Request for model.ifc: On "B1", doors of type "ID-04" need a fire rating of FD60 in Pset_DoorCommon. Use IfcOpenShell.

First a look at what the model holds.

```python
import ifcopenshell
import ifcopenshell.util.element

model = ifcopenshell.open("model.ifc")
print(model.schema)
storey = next(s for s in model.by_type("IfcBuildingStorey") if s.Name == "B1")
doors = [e for e in ifcopenshell.util.element.get_decomposition(storey) if e.is_a("IfcDoor")]
seen = {}
for e in doors:
    element_type = ifcopenshell.util.element.get_type(e)
    key = (element_type.Name if element_type != e and element_type else None, ifcopenshell.util.element.get_pset(e, "Pset_DoorCommon", "FireRating"))
    seen[key] = seen.get(key, 0) + 1
for (name, value), count in sorted(seen.items(), key=str):
    print(count, "x", name, "|", value)
```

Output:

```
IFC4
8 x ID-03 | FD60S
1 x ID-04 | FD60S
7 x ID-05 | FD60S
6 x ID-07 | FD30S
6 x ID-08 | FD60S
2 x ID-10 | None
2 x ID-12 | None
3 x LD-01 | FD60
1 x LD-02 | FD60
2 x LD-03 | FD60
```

```python
import ifcopenshell
import ifcopenshell.api.pset
import ifcopenshell.util.element

model = ifcopenshell.open("model.ifc")

storey = next(s for s in model.by_type("IfcBuildingStorey") if s.Name == "B1")
doors = [e for e in ifcopenshell.util.element.get_decomposition(storey) if e.is_a("IfcDoor")]

count = 0
for e in doors:
    element_type = ifcopenshell.util.element.get_type(e)
    if element_type in (None, e) or element_type.Name != "ID-04":
        continue
    # add_pset returns the element's existing set when there is one.
    pset = ifcopenshell.api.pset.add_pset(model, product=e, name="Pset_DoorCommon")
    ifcopenshell.api.pset.edit_pset(model, pset=pset, properties={"FireRating": "FD60"})
    count += 1

print(count, "doors updated")

model.write("model_v2.ifc")
```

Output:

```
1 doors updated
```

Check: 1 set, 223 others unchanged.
